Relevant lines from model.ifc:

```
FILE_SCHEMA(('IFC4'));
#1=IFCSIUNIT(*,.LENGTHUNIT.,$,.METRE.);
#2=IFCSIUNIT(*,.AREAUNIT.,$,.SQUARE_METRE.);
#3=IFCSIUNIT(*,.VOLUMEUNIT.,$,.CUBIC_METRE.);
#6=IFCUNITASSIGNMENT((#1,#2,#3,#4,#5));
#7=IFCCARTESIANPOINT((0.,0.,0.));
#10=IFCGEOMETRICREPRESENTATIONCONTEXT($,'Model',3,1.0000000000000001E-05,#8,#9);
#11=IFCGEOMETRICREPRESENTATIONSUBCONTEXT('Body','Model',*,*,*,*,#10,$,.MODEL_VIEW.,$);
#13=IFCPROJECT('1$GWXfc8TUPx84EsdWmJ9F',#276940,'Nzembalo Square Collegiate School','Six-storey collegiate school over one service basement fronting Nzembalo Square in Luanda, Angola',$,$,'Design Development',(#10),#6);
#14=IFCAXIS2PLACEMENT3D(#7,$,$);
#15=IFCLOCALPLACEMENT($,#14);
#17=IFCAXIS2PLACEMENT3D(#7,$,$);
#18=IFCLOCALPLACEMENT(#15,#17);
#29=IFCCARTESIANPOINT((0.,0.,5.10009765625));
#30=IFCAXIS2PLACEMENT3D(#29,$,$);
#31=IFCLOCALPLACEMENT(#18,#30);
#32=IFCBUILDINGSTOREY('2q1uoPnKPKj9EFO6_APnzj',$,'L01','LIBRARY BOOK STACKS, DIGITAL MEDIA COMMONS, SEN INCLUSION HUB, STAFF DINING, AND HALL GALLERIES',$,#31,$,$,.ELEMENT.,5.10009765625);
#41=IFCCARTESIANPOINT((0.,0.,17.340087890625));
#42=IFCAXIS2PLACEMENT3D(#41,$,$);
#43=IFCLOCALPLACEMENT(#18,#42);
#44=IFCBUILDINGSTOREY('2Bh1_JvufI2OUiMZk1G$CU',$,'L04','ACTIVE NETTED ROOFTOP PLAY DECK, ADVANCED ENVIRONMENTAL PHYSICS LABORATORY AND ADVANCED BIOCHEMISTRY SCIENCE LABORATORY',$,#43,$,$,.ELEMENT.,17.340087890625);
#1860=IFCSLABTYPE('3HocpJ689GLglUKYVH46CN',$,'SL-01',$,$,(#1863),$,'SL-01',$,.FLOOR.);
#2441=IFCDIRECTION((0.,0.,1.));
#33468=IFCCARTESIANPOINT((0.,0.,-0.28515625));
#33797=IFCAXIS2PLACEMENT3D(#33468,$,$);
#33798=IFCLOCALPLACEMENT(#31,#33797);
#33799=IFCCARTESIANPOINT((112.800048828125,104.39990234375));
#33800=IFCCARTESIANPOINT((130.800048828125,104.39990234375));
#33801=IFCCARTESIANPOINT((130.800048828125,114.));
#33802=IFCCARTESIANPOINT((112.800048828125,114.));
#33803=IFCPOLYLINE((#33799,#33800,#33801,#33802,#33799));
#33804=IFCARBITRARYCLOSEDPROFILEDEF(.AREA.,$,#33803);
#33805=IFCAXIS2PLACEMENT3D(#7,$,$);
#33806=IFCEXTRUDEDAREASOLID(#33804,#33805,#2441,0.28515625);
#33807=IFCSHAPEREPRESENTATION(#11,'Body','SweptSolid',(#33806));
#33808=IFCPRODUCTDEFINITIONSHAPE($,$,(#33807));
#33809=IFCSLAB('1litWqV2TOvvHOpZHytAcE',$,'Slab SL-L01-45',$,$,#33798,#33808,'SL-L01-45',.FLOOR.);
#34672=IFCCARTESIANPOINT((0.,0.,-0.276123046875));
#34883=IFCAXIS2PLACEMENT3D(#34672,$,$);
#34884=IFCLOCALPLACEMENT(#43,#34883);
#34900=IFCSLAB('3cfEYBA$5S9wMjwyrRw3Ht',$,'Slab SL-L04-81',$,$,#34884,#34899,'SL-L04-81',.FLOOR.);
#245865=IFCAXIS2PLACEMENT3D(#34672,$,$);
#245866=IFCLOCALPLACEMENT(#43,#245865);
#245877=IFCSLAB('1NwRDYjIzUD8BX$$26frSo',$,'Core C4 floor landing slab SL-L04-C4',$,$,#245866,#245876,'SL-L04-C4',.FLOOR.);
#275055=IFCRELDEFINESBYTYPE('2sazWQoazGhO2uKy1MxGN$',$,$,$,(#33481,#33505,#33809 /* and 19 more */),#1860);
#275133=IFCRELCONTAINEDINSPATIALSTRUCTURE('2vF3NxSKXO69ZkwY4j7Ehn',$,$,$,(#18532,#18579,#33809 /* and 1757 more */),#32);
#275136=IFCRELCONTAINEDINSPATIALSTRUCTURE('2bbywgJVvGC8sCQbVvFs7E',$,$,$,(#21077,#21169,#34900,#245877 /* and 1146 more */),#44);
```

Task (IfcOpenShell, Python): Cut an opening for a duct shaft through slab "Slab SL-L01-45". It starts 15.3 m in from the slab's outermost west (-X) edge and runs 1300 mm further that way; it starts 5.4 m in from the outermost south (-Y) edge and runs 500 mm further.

```python
import numpy as np
import ifcopenshell
import ifcopenshell.api.feature
import ifcopenshell.api.geometry
import ifcopenshell.api.root
import ifcopenshell.geom
import ifcopenshell.util.placement
import ifcopenshell.util.representation
import ifcopenshell.util.shape
import ifcopenshell.util.unit

model = ifcopenshell.open("model.ifc")
unit_scale = ifcopenshell.util.unit.calculate_unit_scale(model)
settings = ifcopenshell.geom.settings()


def volume(element):
    """Net volume in cubic metres, openings subtracted."""
    shape = ifcopenshell.geom.create_shape(settings, element)
    return ifcopenshell.util.shape.get_volume(shape.geometry)


slab = model.by_id(33809)
before = volume(slab)

# Extent in the slab's own axes, in metres. The edges named are its -X and -Y sides.
slab_shape = ifcopenshell.geom.create_shape(settings, slab)
vertices = ifcopenshell.util.shape.get_vertices(slab_shape.geometry)
x_min, y_min, bottom = vertices.min(axis=0)
top = vertices[:, 2].max()

opening = ifcopenshell.api.root.create_entity(model, ifc_class="IfcOpeningElement", name="Duct shaft opening", predefined_type="OPENING")
context = ifcopenshell.util.representation.get_context(model, "Model", "Body", "MODEL_VIEW")
width, depth = 1.3, 0.5
outline = [(0.0, 0.0), (width, 0.0), (width, depth), (0.0, depth), (0.0, 0.0)]
# Overshoot both faces by 50 mm so the cut is clean.
shape = ifcopenshell.api.geometry.add_slab_representation(
    model, context=context, depth=top - bottom + 0.1, polyline=outline
)
ifcopenshell.api.geometry.assign_representation(model, product=opening, representation=shape)

matrix = ifcopenshell.util.placement.get_local_placement(slab.ObjectPlacement)
matrix[:, 3] = matrix @ np.append(np.array([x_min + 15.3, y_min + 5.4, bottom - 0.05]) / unit_scale, 1.0)
ifcopenshell.api.geometry.edit_object_placement(model, product=opening, matrix=matrix, is_si=False)
ifcopenshell.api.feature.add_feature(model, feature=opening, element=slab)

after = volume(slab)

print(f"slab volume {before:.3f} -> {after:.3f} m3")

model.write("model-out.ifc")
```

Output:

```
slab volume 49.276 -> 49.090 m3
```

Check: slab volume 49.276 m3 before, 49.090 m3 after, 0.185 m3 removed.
